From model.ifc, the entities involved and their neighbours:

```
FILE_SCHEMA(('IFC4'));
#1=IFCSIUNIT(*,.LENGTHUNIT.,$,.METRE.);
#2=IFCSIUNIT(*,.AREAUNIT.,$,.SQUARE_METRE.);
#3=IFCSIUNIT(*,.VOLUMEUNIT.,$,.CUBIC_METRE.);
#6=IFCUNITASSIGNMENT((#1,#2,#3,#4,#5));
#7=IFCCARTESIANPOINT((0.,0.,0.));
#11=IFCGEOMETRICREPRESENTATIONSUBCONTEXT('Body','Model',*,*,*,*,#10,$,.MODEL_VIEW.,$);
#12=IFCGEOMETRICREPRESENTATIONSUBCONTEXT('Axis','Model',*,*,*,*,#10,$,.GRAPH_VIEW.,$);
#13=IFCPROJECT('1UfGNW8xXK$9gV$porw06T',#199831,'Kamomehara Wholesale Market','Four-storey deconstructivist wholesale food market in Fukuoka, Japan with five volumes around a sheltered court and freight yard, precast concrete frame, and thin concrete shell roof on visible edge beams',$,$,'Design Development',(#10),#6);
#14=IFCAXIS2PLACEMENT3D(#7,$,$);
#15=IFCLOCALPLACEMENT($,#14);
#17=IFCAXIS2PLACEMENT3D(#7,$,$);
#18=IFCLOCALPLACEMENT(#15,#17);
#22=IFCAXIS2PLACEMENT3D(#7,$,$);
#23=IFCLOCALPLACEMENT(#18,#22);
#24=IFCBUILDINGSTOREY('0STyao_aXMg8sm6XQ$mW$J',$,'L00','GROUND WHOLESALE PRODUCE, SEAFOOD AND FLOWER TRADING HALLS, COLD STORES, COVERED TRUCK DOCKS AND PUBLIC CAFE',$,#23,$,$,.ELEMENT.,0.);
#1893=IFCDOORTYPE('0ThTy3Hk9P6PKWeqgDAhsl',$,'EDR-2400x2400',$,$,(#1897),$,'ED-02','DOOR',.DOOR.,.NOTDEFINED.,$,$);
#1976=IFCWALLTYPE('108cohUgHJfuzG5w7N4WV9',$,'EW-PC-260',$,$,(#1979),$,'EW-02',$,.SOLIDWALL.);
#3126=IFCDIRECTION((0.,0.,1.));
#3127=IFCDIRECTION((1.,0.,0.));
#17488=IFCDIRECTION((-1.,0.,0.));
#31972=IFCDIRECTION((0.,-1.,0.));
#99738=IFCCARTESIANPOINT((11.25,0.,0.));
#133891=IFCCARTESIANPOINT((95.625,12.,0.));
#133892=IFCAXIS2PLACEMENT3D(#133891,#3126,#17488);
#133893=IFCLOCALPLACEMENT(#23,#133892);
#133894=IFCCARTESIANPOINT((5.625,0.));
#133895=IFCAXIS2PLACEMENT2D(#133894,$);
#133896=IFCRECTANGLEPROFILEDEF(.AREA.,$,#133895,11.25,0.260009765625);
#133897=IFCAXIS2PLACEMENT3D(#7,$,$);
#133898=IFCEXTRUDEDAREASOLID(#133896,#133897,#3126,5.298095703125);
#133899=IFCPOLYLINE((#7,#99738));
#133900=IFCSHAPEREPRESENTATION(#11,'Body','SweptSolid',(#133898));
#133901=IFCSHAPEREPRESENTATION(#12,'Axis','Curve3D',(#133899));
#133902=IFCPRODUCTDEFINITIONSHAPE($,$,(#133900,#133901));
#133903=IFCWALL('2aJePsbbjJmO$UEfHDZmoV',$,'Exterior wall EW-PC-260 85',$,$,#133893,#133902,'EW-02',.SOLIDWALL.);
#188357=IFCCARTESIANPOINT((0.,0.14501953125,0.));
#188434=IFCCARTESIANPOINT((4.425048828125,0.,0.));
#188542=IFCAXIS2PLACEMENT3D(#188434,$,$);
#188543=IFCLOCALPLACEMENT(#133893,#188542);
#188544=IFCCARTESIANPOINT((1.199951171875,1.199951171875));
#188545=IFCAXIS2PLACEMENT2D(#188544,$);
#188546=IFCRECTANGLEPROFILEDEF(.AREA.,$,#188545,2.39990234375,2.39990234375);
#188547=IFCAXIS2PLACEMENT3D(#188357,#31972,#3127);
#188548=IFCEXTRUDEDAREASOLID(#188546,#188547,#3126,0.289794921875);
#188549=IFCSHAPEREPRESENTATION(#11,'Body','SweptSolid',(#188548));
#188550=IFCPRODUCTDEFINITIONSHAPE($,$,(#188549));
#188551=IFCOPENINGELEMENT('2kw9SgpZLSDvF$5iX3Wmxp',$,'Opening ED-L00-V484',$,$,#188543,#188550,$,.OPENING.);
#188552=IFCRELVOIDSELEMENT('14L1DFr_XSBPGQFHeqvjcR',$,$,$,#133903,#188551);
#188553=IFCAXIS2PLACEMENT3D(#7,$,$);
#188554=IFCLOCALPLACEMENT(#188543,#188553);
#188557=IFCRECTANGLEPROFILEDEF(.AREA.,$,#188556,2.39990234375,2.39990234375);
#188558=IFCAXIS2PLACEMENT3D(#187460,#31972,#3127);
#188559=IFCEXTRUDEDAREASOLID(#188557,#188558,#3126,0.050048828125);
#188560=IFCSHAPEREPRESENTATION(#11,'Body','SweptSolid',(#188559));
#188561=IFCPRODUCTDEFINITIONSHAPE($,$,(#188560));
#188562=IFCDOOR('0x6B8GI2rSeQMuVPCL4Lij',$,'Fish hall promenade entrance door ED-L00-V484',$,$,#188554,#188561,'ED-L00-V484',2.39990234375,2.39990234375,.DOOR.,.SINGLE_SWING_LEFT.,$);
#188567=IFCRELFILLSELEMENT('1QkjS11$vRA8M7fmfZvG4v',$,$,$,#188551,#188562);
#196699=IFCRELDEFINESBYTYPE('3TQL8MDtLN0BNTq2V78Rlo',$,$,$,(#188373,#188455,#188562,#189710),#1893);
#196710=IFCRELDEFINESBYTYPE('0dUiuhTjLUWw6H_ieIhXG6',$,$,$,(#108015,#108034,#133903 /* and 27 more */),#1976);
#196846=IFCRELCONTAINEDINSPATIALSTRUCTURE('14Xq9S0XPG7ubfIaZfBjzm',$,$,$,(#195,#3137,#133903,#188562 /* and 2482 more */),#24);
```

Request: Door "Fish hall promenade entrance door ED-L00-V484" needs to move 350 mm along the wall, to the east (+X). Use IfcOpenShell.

```python
import ifcopenshell
import ifcopenshell.api.geometry
import ifcopenshell.util.placement

model = ifcopenshell.open("model.ifc")

door = model.by_guid("0x6B8GI2rSeQMuVPCL4Lij")
opening = door.FillsVoids[0].RelatingOpeningElement
wall = opening.VoidsElements[0].RelatingBuildingElement

wall_matrix = ifcopenshell.util.placement.get_local_placement(wall.ObjectPlacement)
shift = wall_matrix[:3, 0] * -0.35
before = ifcopenshell.util.placement.get_local_placement(door.ObjectPlacement)[:3, 3].copy()

# The door is placed relative to its opening, so it follows when the opening moves.
matrix = ifcopenshell.util.placement.get_local_placement(opening.ObjectPlacement)
matrix[:3, 3] += shift
ifcopenshell.api.geometry.edit_object_placement(
    model, product=opening, matrix=matrix, is_si=False, should_transform_children=True
)

after = ifcopenshell.util.placement.get_local_placement(door.ObjectPlacement)[:3, 3]
print("door moved by", (after - before).round(3) + 0.0)

model.write("model_rev.ifc")
```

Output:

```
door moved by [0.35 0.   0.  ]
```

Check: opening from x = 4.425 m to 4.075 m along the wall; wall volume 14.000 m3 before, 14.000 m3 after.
